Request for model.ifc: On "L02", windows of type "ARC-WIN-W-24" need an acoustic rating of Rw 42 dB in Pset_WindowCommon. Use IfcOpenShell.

First a look at what the model holds.

```python
import ifcopenshell
import ifcopenshell.util.element

model = ifcopenshell.open("model.ifc")
print(model.schema)
storey = next(s for s in model.by_type("IfcBuildingStorey") if s.Name == "L02")
windows = [e for e in ifcopenshell.util.element.get_decomposition(storey) if e.is_a("IfcWindow")]
seen = {}
for e in windows:
    element_type = ifcopenshell.util.element.get_type(e)
    key = (element_type.Name if element_type != e and element_type else None, ifcopenshell.util.element.get_pset(e, "Pset_WindowCommon", "AcousticRating"))
    seen[key] = seen.get(key, 0) + 1
for (name, value), count in sorted(seen.items(), key=str):
    print(count, "x", name, "|", value)
```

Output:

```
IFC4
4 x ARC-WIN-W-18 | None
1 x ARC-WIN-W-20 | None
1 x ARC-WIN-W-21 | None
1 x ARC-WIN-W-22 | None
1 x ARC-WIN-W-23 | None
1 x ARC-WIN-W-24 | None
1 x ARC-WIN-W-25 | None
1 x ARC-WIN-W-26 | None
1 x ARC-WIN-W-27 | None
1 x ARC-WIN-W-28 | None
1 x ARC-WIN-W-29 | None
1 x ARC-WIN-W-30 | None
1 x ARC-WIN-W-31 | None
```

```python
import ifcopenshell
import ifcopenshell.api.pset
import ifcopenshell.util.element

model = ifcopenshell.open("model.ifc")

storey = next(s for s in model.by_type("IfcBuildingStorey") if s.Name == "L02")
windows = [e for e in ifcopenshell.util.element.get_decomposition(storey) if e.is_a("IfcWindow")]

count = 0
for e in windows:
    element_type = ifcopenshell.util.element.get_type(e)
    if element_type in (None, e) or element_type.Name != "ARC-WIN-W-24":
        continue
    # add_pset returns the element's existing set when there is one.
    pset = ifcopenshell.api.pset.add_pset(model, product=e, name="Pset_WindowCommon")
    ifcopenshell.api.pset.edit_pset(model, pset=pset, properties={"AcousticRating": "Rw 42 dB"})
    count += 1

print(count, "windows updated")

model.write("model-out.ifc")
```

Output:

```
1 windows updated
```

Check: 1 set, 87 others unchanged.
